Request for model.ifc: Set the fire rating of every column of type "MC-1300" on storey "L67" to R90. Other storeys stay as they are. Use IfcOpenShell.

First a look at what the model holds.

```python
import ifcopenshell
import ifcopenshell.util.element

model = ifcopenshell.open("model.ifc")
print(model.schema)
storey = next(s for s in model.by_type("IfcBuildingStorey") if s.Name == "L67")
columns = [e for e in ifcopenshell.util.element.get_decomposition(storey) if e.is_a("IfcColumn")]
seen = {}
for e in columns:
    element_type = ifcopenshell.util.element.get_type(e)
    key = (element_type.Name if element_type != e and element_type else None, ifcopenshell.util.element.get_pset(e, "Pset_ColumnCommon", "FireRating"))
    seen[key] = seen.get(key, 0) + 1
for (name, value), count in sorted(seen.items(), key=str):
    print(count, "x", name, "|", value)
```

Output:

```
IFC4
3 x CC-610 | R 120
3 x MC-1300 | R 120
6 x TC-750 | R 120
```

```python
import ifcopenshell
import ifcopenshell.api.pset
import ifcopenshell.util.element

model = ifcopenshell.open("model.ifc")

storey = next(s for s in model.by_type("IfcBuildingStorey") if s.Name == "L67")
columns = [e for e in ifcopenshell.util.element.get_decomposition(storey) if e.is_a("IfcColumn")]

count = 0
for e in columns:
    element_type = ifcopenshell.util.element.get_type(e)
    if element_type in (None, e) or element_type.Name != "MC-1300":
        continue
    found = ifcopenshell.util.element.get_pset(e, "Pset_ColumnCommon", should_inherit=False)
    if found:
        pset = model.by_id(found["id"])
        if len(ifcopenshell.util.element.get_elements_by_pset(pset)) > 1:
            pset = ifcopenshell.api.pset.unshare_pset(model, products=[e], pset=pset)[0]
    else:
        pset = ifcopenshell.api.pset.add_pset(model, product=e, name="Pset_ColumnCommon")
    ifcopenshell.api.pset.edit_pset(model, pset=pset, properties={"FireRating": "R90"})
    count += 1

print(count, "columns updated")

model.write("model_updated.ifc")
```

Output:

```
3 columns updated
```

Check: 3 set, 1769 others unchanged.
